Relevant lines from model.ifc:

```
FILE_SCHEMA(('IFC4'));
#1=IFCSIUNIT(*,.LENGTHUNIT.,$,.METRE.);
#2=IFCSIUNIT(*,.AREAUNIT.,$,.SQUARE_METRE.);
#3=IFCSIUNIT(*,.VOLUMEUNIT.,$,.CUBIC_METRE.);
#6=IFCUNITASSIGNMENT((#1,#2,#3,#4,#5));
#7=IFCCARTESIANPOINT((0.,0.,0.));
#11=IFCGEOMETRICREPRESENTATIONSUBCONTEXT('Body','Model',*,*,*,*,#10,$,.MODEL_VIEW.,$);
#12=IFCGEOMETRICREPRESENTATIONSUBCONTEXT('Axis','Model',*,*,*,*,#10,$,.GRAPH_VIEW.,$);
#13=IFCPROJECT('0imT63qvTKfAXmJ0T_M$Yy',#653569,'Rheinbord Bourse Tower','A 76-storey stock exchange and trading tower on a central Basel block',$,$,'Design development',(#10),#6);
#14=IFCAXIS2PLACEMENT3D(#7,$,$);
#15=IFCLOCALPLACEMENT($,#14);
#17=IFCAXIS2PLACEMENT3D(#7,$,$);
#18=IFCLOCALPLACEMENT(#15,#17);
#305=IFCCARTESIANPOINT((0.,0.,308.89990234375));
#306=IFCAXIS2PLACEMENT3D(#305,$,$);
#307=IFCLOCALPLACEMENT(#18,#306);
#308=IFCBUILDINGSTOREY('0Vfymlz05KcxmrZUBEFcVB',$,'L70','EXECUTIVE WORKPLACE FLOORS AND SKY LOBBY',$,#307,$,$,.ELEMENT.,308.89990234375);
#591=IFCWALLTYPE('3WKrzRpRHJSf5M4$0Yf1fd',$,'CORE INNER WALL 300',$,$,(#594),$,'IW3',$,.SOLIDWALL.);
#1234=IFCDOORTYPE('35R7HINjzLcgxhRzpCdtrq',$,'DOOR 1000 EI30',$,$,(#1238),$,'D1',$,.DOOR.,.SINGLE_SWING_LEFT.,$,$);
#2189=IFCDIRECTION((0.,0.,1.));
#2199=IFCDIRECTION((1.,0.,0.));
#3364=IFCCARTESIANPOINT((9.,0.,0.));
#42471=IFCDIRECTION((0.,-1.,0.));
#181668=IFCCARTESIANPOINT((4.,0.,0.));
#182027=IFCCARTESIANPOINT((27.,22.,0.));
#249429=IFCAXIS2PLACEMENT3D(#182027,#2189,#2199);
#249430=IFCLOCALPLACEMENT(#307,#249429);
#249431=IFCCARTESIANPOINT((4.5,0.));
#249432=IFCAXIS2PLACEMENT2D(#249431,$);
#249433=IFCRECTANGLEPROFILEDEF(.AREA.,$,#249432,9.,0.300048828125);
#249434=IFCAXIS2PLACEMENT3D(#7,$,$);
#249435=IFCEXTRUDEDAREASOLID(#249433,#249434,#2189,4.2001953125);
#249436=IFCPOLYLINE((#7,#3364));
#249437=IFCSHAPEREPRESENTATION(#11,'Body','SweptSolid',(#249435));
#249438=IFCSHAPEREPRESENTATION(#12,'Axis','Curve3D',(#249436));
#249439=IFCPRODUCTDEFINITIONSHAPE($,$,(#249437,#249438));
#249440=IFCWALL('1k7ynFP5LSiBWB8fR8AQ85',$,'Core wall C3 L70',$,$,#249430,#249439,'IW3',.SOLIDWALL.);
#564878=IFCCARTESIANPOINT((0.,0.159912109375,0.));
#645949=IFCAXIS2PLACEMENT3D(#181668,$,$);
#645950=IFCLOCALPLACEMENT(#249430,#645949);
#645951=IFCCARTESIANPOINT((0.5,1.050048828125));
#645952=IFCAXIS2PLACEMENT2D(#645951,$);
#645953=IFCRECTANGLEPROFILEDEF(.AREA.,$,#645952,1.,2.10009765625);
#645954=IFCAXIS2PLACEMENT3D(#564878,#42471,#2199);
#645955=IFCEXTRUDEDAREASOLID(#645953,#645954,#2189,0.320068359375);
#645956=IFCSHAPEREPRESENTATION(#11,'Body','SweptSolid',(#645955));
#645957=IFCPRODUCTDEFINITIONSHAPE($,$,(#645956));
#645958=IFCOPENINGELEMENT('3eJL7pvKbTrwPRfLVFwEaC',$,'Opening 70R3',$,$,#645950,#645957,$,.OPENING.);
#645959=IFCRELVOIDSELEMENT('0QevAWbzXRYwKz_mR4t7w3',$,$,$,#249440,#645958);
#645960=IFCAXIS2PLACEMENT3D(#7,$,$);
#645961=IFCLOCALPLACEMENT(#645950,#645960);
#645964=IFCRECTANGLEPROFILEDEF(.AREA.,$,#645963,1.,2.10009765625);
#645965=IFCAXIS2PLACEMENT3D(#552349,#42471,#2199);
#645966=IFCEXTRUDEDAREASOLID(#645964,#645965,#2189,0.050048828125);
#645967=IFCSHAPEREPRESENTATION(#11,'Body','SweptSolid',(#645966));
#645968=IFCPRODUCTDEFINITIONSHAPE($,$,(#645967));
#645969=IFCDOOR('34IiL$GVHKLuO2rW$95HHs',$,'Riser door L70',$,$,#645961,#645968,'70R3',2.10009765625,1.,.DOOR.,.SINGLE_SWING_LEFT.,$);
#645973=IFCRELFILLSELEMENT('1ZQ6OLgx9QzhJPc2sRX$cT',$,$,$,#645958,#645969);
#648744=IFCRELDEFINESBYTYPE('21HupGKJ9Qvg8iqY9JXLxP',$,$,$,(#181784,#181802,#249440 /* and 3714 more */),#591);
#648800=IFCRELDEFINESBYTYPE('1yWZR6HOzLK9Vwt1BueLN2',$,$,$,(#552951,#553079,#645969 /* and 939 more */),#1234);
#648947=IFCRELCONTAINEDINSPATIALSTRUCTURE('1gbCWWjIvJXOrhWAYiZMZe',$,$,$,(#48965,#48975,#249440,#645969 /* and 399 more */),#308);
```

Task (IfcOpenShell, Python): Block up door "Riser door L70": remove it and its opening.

```python
import ifcopenshell
import ifcopenshell.api.feature
import ifcopenshell.api.root
import ifcopenshell.geom
import ifcopenshell.util.shape

model = ifcopenshell.open("model.ifc")
settings = ifcopenshell.geom.settings()


def volume(element):
    """Net volume in cubic metres, openings subtracted."""
    shape = ifcopenshell.geom.create_shape(settings, element)
    return ifcopenshell.util.shape.get_volume(shape.geometry)


door = model.by_guid("34IiL$GVHKLuO2rW$95HHs")
opening = door.FillsVoids[0].RelatingOpeningElement
wall = opening.VoidsElements[0].RelatingBuildingElement
before = volume(wall)

ifcopenshell.api.root.remove_product(model, product=door)
ifcopenshell.api.feature.remove_feature(model, feature=opening)

after = volume(wall)

print(f"wall volume {before:.3f} -> {after:.3f} m3")

model.write("model_updated.ifc")
```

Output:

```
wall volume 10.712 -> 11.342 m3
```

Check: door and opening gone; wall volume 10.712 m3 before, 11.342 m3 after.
